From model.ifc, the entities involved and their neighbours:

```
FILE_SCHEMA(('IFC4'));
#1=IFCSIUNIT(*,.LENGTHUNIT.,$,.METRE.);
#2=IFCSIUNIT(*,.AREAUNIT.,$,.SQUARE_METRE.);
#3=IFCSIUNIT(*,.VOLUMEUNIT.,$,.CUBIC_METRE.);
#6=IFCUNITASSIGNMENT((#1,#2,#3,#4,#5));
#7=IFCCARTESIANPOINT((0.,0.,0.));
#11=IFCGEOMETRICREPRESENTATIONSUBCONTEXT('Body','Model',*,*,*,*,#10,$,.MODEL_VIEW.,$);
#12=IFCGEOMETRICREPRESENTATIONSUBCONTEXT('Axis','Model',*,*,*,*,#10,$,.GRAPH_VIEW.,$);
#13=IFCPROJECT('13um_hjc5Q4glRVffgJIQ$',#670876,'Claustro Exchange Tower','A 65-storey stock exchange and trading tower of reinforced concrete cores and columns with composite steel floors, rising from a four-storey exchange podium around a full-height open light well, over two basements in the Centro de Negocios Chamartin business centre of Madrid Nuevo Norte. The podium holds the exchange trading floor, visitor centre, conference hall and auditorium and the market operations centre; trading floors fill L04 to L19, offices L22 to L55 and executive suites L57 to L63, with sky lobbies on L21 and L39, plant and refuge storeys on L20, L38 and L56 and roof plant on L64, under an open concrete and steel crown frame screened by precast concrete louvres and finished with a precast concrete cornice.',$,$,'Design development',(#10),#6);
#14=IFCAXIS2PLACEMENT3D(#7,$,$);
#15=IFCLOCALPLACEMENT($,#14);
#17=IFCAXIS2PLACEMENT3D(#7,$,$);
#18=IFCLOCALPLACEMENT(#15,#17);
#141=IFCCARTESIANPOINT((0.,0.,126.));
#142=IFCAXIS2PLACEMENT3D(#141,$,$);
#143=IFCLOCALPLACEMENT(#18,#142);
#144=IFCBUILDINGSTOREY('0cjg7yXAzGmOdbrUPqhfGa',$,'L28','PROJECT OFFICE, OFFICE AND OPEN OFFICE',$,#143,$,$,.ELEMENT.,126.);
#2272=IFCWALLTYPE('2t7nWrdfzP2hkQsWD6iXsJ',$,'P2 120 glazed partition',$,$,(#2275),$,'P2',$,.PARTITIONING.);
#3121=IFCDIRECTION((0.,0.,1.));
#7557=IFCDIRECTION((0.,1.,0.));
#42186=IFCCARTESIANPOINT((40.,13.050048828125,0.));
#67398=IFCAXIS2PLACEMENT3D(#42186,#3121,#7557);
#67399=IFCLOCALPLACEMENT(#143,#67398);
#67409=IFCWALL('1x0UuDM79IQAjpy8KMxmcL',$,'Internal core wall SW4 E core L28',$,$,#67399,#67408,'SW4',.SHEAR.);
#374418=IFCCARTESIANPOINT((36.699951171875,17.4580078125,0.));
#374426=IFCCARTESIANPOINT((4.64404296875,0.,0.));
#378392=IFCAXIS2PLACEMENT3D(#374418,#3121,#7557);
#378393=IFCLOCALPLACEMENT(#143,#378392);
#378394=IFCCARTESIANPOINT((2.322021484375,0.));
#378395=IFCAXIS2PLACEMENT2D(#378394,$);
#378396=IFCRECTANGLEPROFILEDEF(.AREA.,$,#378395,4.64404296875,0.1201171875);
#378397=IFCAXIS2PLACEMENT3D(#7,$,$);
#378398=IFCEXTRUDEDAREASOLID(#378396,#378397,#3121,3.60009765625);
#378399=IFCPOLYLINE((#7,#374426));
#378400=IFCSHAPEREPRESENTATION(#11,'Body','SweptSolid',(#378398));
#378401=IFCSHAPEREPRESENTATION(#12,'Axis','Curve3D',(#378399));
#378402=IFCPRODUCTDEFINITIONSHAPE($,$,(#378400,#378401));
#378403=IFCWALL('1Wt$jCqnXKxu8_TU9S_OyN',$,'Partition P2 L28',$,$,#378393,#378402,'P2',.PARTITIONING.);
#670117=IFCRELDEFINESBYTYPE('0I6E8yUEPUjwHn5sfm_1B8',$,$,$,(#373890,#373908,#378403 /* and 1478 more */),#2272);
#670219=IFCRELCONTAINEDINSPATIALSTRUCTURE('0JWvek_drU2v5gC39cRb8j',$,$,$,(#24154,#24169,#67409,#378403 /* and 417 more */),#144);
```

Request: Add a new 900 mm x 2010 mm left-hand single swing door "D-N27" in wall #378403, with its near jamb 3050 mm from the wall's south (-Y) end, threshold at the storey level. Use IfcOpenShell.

```python
import numpy as np
import ifcopenshell
import ifcopenshell.api.feature
import ifcopenshell.api.geometry
import ifcopenshell.api.root
import ifcopenshell.api.spatial
import ifcopenshell.geom
import ifcopenshell.util.element
import ifcopenshell.util.placement
import ifcopenshell.util.representation
import ifcopenshell.util.shape
import ifcopenshell.util.unit

model = ifcopenshell.open("model.ifc")
unit_scale = ifcopenshell.util.unit.calculate_unit_scale(model)
settings = ifcopenshell.geom.settings()


def volume(element):
    """Net volume in cubic metres, openings subtracted."""
    shape = ifcopenshell.geom.create_shape(settings, element)
    return ifcopenshell.util.shape.get_volume(shape.geometry)


wall = model.by_guid("1Wt$jCqnXKxu8_TU9S_OyN")
storey = ifcopenshell.util.element.get_container(wall, ifc_class="IfcBuildingStorey")
context = ifcopenshell.util.representation.get_context(model, "Model", "Body", "MODEL_VIEW")
before = volume(wall)

width, height, from_end, sill = 0.9, 2.01, 3.05, 0.0  # metres

# The wall runs along its own X axis, and the end named is its -X end.
wall_shape = ifcopenshell.geom.create_shape(settings, wall)
x, y, z = ifcopenshell.util.shape.get_vertices(wall_shape.geometry).T
start = x.min() + from_end
face, thickness = float(y.min()), float(y.max() - y.min())
wall_matrix = ifcopenshell.util.placement.get_local_placement(wall.ObjectPlacement)
level = ifcopenshell.util.placement.get_local_placement(storey.ObjectPlacement)[2, 3]


def in_wall(x, y):
    """Placement at x, y metres in the wall's axes, at sill height."""
    matrix = wall_matrix.copy()
    matrix[:, 3] = wall_matrix @ np.array([x / unit_scale, y / unit_scale, 0.0, 1.0])
    matrix[2, 3] = level + sill / unit_scale
    return matrix


# Opening: a box that overshoots both wall faces by 50 mm.
opening = ifcopenshell.api.root.create_entity(model, ifc_class="IfcOpeningElement", predefined_type="OPENING")
box = ifcopenshell.api.geometry.add_wall_representation(
    model, context=context, length=width, height=height, thickness=thickness + 0.1
)
ifcopenshell.api.geometry.assign_representation(model, product=opening, representation=box)
ifcopenshell.api.geometry.edit_object_placement(model, product=opening, matrix=in_wall(start, face - 0.05), is_si=False)
ifcopenshell.api.feature.add_feature(model, feature=opening, element=wall)

door = ifcopenshell.api.root.create_entity(model, ifc_class="IfcDoor", name="D-N27", predefined_type="DOOR")
door.OverallWidth, door.OverallHeight = width / unit_scale, height / unit_scale
door.OperationType = "SINGLE_SWING_LEFT"
body = ifcopenshell.api.geometry.add_door_representation(
    model,
    context=context,
    overall_width=door.OverallWidth,
    overall_height=door.OverallHeight,
    operation_type="SINGLE_SWING_LEFT",
    lining_properties={"LiningDepth": thickness / unit_scale, "ThresholdDepth": thickness / unit_scale},
)
ifcopenshell.api.geometry.assign_representation(model, product=door, representation=body)
ifcopenshell.api.spatial.assign_container(model, products=[door], relating_structure=storey)
ifcopenshell.api.feature.add_filling(model, opening=opening, element=door)

# The lining spans the wall, so the door starts at the wall face.
ifcopenshell.api.geometry.edit_object_placement(model, product=door, matrix=in_wall(start, face), is_si=False)

after = volume(wall)

print(f"wall volume {before:.3f} -> {after:.3f} m3")

model.write("model_rev.ifc")
```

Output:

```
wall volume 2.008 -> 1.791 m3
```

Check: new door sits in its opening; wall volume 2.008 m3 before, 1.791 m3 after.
